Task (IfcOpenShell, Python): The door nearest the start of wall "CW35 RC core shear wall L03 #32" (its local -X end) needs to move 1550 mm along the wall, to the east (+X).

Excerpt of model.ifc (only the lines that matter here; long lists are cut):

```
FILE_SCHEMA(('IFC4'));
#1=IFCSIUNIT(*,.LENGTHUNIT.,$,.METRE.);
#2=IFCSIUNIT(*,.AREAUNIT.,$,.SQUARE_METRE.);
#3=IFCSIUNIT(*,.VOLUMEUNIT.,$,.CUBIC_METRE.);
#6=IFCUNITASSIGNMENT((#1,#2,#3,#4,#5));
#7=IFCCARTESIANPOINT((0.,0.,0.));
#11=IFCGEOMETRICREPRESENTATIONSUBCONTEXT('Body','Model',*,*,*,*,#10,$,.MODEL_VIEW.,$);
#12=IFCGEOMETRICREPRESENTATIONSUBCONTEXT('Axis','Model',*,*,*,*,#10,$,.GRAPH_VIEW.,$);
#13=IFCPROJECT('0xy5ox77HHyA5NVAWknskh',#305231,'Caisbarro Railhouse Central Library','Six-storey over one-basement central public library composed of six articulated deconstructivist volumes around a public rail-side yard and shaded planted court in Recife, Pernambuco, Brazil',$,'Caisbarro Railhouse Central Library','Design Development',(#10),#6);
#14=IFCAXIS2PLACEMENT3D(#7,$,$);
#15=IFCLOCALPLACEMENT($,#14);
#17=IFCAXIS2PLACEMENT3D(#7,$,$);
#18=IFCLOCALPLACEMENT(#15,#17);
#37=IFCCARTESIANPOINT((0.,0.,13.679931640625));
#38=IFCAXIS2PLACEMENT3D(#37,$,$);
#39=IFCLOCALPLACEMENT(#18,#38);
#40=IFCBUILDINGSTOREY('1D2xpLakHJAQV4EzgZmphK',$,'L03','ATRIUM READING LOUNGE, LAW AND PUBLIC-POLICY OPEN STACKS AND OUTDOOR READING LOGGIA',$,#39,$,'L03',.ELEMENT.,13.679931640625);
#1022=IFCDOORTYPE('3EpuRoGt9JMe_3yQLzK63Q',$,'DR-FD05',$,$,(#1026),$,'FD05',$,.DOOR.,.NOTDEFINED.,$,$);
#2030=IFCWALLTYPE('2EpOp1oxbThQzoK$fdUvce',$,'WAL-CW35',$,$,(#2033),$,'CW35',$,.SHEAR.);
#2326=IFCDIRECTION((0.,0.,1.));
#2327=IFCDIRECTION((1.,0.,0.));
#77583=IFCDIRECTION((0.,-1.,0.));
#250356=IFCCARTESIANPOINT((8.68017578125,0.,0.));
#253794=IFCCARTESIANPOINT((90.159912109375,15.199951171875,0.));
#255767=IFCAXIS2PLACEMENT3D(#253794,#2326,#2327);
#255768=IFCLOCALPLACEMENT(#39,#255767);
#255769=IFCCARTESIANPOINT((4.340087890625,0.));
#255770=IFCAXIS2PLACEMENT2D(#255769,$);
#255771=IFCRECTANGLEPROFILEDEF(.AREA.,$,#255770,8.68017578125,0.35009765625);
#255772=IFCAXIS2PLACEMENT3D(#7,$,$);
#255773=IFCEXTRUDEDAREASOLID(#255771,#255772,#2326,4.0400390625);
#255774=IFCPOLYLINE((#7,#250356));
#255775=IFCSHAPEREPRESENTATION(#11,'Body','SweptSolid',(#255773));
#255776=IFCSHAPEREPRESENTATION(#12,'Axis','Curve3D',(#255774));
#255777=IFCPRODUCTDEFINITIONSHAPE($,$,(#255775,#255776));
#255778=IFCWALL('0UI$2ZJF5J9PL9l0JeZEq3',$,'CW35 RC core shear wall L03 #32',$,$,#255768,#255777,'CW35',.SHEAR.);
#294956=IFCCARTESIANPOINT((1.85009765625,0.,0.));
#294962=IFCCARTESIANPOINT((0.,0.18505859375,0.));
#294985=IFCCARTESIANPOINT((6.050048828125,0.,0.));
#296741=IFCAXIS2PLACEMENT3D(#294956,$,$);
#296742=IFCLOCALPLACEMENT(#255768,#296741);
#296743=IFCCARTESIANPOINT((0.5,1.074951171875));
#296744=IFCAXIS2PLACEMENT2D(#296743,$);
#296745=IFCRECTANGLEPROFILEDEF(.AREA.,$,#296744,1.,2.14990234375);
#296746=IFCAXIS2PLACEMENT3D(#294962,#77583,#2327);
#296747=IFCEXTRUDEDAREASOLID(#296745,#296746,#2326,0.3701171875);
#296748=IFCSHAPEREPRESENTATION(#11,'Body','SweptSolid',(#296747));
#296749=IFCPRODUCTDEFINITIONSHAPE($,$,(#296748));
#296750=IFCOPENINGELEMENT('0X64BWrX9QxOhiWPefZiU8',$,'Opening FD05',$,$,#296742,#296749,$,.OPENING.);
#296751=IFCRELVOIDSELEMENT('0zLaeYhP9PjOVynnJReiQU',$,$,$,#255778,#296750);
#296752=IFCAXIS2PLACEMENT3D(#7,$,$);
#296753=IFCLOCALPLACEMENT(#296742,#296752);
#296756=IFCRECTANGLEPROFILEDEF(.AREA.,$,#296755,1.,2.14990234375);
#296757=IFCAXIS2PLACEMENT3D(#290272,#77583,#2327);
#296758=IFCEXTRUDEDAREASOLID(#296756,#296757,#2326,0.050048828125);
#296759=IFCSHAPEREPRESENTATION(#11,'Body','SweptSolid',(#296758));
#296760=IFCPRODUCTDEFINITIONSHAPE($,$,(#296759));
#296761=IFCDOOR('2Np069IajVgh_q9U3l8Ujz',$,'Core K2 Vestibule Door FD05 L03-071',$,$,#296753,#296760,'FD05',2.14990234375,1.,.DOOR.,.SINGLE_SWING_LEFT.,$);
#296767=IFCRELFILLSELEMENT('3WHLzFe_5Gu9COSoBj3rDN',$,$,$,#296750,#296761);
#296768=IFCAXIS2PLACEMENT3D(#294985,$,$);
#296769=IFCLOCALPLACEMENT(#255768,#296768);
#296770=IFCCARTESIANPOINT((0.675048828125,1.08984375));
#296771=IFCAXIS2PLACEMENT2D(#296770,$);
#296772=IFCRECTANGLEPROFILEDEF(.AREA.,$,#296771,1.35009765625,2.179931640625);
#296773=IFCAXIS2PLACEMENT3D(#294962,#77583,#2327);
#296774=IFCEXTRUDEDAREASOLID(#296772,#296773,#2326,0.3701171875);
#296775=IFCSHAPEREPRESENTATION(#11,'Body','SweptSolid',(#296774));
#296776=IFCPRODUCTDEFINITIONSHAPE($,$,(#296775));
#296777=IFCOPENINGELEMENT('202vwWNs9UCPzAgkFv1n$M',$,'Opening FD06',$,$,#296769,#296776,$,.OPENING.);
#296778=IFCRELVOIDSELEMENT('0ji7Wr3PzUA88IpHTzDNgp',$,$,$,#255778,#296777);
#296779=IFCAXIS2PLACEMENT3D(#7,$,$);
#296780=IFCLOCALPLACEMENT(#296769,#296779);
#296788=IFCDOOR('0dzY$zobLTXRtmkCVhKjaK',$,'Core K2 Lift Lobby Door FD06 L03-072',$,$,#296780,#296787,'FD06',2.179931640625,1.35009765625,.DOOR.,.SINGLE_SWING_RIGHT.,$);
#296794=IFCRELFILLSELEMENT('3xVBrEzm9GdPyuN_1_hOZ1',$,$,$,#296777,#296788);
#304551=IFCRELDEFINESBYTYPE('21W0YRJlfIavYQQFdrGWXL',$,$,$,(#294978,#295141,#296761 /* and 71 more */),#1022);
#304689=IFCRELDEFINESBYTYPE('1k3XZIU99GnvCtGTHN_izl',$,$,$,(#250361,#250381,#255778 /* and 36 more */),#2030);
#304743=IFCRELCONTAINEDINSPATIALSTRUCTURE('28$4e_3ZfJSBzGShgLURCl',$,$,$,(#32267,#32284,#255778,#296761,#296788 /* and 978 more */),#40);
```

```python
import ifcopenshell
import ifcopenshell.api.geometry
import ifcopenshell.util.placement
import ifcopenshell.util.unit

model = ifcopenshell.open("model.ifc")
unit_scale = ifcopenshell.util.unit.calculate_unit_scale(model)

door = model.by_id(296761)
opening = door.FillsVoids[0].RelatingOpeningElement
wall = opening.VoidsElements[0].RelatingBuildingElement

wall_matrix = ifcopenshell.util.placement.get_local_placement(wall.ObjectPlacement)
shift = wall_matrix[:3, 0] * 1.55 / unit_scale
before = ifcopenshell.util.placement.get_local_placement(door.ObjectPlacement)[:3, 3].copy()

# The door is placed relative to its opening, so it follows when the opening moves.
matrix = ifcopenshell.util.placement.get_local_placement(opening.ObjectPlacement)
matrix[:3, 3] += shift
ifcopenshell.api.geometry.edit_object_placement(
    model, product=opening, matrix=matrix, is_si=False, should_transform_children=True
)

after = ifcopenshell.util.placement.get_local_placement(door.ObjectPlacement)[:3, 3]
print("door moved by", (after - before).round(3) + 0.0)

model.write("model_edited.ifc")
```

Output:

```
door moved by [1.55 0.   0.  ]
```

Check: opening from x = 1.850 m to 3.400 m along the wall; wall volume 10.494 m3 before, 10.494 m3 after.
